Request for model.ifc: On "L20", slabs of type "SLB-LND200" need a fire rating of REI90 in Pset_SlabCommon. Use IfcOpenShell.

First a look at what the model holds.

```python
import ifcopenshell
import ifcopenshell.util.element

model = ifcopenshell.open("model.ifc")
print(model.schema)
storey = next(s for s in model.by_type("IfcBuildingStorey") if s.Name == "L20")
slabs = [e for e in ifcopenshell.util.element.get_decomposition(storey) if e.is_a("IfcSlab")]
seen = {}
for e in slabs:
    element_type = ifcopenshell.util.element.get_type(e)
    key = (element_type.Name if element_type != e and element_type else None, ifcopenshell.util.element.get_pset(e, "Pset_SlabCommon", "FireRating"))
    seen[key] = seen.get(key, 0) + 1
for (name, value), count in sorted(seen.items(), key=str):
    print(count, "x", name, "|", value)
```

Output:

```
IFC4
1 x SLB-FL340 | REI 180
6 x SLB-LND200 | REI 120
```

```python
import ifcopenshell
import ifcopenshell.api.pset
import ifcopenshell.util.element

model = ifcopenshell.open("model.ifc")

storey = next(s for s in model.by_type("IfcBuildingStorey") if s.Name == "L20")
slabs = [e for e in ifcopenshell.util.element.get_decomposition(storey) if e.is_a("IfcSlab")]

count = 0
for e in slabs:
    element_type = ifcopenshell.util.element.get_type(e)
    if element_type in (None, e) or element_type.Name != "SLB-LND200":
        continue
    # add_pset returns the element's existing set when there is one.
    pset = ifcopenshell.api.pset.add_pset(model, product=e, name="Pset_SlabCommon")
    ifcopenshell.api.pset.edit_pset(model, pset=pset, properties={"FireRating": "REI90"})
    count += 1

print(count, "slabs updated")

model.write("model_v2.ifc")
```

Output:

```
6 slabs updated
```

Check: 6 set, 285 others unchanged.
